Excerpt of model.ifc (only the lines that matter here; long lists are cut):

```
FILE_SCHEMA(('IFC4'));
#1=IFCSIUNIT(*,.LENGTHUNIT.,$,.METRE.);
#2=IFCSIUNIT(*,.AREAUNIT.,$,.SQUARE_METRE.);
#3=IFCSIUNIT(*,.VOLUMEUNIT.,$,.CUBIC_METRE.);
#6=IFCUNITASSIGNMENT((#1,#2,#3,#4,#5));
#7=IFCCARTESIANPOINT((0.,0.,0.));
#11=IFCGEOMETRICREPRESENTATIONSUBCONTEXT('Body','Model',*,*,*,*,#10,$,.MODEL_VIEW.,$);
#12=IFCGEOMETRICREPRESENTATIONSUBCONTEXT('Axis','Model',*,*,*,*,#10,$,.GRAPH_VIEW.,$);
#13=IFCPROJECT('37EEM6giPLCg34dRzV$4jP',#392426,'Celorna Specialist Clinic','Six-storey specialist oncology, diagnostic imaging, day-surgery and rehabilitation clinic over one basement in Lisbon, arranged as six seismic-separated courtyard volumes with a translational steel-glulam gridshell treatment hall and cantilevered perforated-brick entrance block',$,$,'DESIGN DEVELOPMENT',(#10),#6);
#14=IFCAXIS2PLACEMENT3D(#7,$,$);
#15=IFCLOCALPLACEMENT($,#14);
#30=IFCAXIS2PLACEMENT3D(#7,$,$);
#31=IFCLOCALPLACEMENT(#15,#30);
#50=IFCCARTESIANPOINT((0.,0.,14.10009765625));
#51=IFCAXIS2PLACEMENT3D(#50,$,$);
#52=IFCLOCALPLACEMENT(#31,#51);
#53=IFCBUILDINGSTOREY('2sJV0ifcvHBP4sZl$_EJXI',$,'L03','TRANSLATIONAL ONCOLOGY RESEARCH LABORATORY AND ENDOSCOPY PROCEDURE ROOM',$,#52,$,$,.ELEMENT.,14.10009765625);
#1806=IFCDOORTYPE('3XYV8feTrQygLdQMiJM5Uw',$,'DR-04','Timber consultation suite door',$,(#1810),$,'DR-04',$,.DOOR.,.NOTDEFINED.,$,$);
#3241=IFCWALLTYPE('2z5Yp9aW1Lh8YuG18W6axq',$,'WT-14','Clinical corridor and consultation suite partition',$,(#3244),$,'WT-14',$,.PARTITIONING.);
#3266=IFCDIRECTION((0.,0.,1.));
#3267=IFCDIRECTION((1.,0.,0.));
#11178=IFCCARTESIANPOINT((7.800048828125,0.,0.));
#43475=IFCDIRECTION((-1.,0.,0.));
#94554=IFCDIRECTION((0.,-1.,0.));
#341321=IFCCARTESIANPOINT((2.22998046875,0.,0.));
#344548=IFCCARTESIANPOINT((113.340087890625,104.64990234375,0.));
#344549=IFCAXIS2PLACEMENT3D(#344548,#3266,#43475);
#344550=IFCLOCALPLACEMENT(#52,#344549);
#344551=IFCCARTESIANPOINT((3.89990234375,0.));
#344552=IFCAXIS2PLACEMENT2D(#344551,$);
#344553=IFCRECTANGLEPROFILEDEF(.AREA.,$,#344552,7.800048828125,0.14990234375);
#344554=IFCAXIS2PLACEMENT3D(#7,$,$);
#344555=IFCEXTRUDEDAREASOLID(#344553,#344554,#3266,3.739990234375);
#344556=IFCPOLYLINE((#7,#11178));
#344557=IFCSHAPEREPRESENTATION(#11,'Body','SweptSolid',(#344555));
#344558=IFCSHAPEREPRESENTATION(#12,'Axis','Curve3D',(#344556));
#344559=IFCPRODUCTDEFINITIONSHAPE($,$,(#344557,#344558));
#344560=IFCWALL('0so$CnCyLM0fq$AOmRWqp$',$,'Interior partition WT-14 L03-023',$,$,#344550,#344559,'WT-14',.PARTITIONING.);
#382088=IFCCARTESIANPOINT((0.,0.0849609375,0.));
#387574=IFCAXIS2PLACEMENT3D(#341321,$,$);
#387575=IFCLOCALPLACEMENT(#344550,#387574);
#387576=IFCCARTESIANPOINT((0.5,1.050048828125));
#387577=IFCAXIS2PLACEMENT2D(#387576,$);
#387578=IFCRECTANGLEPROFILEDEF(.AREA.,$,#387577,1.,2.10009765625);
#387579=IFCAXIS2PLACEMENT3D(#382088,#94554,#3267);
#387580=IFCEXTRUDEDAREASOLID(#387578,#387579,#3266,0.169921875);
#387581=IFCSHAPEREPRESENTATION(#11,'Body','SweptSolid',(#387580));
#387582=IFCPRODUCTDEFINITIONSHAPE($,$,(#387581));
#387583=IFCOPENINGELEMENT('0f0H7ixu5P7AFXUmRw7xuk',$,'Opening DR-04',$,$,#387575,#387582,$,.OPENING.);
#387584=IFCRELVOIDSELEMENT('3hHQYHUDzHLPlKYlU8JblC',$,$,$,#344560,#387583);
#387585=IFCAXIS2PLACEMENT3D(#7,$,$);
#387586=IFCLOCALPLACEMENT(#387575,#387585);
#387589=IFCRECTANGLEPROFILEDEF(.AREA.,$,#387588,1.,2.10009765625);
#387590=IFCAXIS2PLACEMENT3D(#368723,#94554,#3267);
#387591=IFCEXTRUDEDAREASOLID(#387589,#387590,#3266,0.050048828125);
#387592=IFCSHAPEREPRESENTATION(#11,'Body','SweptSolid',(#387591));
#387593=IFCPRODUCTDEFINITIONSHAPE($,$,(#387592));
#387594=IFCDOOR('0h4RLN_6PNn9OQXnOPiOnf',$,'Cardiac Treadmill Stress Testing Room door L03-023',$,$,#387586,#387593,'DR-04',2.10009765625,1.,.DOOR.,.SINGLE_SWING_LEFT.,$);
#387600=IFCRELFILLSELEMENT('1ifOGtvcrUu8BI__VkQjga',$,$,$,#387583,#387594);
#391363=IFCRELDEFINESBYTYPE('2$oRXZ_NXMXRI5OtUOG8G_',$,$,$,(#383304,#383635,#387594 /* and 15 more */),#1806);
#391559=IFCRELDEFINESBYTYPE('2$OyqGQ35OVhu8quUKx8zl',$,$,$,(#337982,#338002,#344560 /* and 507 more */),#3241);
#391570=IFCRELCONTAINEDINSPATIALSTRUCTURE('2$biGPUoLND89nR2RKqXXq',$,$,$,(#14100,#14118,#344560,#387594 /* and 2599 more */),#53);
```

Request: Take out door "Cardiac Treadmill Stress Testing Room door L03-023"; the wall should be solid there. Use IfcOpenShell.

```python
import ifcopenshell
import ifcopenshell.api.feature
import ifcopenshell.api.root
import ifcopenshell.geom
import ifcopenshell.util.shape

model = ifcopenshell.open("model.ifc")
settings = ifcopenshell.geom.settings()


def volume(element):
    """Net volume in cubic metres, openings subtracted."""
    shape = ifcopenshell.geom.create_shape(settings, element)
    return ifcopenshell.util.shape.get_volume(shape.geometry)


door = model.by_guid("0h4RLN_6PNn9OQXnOPiOnf")
opening = door.FillsVoids[0].RelatingOpeningElement
wall = opening.VoidsElements[0].RelatingBuildingElement
before = volume(wall)

ifcopenshell.api.root.remove_product(model, product=door)
ifcopenshell.api.feature.remove_feature(model, feature=opening)

after = volume(wall)

print(f"wall volume {before:.3f} -> {after:.3f} m3")

model.write("model_edited.ifc")
```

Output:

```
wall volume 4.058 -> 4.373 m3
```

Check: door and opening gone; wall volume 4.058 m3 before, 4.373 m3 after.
